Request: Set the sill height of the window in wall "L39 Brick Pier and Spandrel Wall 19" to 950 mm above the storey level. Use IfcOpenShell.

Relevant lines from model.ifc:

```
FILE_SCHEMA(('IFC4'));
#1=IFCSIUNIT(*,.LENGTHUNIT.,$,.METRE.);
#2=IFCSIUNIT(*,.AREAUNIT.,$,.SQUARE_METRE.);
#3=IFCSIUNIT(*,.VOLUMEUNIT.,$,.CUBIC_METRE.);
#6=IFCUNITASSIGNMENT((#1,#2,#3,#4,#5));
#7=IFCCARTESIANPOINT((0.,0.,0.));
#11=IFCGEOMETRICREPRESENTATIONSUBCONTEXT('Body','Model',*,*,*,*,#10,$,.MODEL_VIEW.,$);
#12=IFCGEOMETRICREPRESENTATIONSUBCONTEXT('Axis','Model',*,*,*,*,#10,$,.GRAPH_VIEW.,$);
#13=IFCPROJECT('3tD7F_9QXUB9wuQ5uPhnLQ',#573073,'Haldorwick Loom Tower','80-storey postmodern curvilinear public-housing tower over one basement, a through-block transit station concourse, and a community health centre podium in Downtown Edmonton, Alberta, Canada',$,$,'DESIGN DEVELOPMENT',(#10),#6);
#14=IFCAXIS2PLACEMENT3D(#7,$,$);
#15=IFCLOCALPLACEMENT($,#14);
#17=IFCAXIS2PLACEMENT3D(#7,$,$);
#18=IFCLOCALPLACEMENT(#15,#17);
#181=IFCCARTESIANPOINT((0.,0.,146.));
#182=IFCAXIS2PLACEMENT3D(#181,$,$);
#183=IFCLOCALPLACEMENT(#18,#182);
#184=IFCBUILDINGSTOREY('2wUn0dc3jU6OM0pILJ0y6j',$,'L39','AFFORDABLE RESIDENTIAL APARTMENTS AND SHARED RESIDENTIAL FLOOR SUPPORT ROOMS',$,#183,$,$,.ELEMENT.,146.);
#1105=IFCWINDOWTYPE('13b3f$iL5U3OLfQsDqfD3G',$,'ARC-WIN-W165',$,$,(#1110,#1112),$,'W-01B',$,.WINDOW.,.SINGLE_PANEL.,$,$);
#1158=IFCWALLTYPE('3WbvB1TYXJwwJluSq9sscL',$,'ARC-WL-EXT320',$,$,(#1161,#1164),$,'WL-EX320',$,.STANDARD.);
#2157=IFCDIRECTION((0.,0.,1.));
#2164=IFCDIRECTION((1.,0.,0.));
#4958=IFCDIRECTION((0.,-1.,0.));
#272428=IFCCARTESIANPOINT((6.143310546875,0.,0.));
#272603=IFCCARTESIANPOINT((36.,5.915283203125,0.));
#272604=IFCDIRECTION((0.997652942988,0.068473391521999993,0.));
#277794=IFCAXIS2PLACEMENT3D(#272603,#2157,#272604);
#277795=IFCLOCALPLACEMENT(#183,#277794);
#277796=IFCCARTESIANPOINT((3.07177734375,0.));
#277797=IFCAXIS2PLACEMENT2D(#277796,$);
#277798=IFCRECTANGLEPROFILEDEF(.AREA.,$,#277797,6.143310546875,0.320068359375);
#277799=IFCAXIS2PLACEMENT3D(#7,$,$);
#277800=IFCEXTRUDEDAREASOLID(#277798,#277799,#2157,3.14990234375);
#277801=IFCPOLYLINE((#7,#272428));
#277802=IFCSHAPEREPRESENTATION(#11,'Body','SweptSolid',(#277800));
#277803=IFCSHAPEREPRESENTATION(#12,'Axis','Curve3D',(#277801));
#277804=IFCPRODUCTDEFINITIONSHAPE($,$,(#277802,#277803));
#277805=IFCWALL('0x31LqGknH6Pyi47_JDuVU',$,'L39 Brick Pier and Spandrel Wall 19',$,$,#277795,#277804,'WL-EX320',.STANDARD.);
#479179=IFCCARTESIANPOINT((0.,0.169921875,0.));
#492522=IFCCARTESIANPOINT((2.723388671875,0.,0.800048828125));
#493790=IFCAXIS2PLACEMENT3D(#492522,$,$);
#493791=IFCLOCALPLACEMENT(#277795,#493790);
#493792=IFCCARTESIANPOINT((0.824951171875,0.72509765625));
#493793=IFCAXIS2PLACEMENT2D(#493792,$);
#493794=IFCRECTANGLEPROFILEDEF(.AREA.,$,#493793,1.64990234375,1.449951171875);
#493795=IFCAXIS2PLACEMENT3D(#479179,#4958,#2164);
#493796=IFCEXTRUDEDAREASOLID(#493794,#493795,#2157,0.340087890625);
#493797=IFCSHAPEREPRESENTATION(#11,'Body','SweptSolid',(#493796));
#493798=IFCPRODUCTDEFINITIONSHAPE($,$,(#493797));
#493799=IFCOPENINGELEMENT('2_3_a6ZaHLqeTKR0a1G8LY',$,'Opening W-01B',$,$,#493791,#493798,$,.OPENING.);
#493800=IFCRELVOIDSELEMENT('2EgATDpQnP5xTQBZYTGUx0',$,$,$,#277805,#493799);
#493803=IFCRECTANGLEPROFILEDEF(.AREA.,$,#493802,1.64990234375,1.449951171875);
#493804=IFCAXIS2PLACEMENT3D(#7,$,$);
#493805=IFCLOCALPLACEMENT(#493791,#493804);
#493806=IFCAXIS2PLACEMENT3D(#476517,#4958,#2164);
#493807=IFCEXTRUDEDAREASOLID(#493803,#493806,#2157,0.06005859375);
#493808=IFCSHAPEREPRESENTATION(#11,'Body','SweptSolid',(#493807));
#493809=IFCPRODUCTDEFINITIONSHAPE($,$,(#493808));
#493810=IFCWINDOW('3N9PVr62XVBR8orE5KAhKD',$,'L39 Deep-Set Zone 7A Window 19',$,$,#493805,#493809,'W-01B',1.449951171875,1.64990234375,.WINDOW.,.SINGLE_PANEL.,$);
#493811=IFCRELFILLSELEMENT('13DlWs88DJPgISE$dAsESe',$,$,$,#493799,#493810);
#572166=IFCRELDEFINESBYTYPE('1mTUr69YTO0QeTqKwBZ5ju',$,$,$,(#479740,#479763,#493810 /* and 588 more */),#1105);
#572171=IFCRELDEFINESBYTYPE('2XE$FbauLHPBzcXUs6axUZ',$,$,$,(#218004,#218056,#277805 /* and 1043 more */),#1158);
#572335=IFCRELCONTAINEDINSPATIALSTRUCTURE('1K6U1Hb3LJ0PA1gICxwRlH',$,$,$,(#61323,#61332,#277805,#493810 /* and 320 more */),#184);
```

```python
import numpy as np
import ifcopenshell
import ifcopenshell.api.geometry
import ifcopenshell.geom
import ifcopenshell.util.element
import ifcopenshell.util.placement
import ifcopenshell.util.shape
import ifcopenshell.util.unit

model = ifcopenshell.open("model.ifc")
unit_scale = ifcopenshell.util.unit.calculate_unit_scale(model)

window = model.by_id(493810)
opening = window.FillsVoids[0].RelatingOpeningElement
storey = ifcopenshell.util.element.get_container(window, ifc_class="IfcBuildingStorey")
level = ifcopenshell.util.placement.get_local_placement(storey.ObjectPlacement)[2, 3]

# The opening's origin need not be at the sill, so measure its lowest point.
shape = ifcopenshell.geom.create_shape(ifcopenshell.geom.settings(), opening)
bottom = ifcopenshell.util.shape.get_shape_bottom_elevation(shape, shape.geometry) / unit_scale
dz = level + 0.95 / unit_scale - bottom

shift = np.array([0.0, 0.0, dz])
# The window is placed relative to its opening, so it follows when the opening moves.
matrix = ifcopenshell.util.placement.get_local_placement(opening.ObjectPlacement)
matrix[:3, 3] += shift
ifcopenshell.api.geometry.edit_object_placement(
    model, product=opening, matrix=matrix, is_si=False, should_transform_children=True
)

print(f"moved by {dz * unit_scale:+.3f} m")

model.write("model_rev.ifc")
```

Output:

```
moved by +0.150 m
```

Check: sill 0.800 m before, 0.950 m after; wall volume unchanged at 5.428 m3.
